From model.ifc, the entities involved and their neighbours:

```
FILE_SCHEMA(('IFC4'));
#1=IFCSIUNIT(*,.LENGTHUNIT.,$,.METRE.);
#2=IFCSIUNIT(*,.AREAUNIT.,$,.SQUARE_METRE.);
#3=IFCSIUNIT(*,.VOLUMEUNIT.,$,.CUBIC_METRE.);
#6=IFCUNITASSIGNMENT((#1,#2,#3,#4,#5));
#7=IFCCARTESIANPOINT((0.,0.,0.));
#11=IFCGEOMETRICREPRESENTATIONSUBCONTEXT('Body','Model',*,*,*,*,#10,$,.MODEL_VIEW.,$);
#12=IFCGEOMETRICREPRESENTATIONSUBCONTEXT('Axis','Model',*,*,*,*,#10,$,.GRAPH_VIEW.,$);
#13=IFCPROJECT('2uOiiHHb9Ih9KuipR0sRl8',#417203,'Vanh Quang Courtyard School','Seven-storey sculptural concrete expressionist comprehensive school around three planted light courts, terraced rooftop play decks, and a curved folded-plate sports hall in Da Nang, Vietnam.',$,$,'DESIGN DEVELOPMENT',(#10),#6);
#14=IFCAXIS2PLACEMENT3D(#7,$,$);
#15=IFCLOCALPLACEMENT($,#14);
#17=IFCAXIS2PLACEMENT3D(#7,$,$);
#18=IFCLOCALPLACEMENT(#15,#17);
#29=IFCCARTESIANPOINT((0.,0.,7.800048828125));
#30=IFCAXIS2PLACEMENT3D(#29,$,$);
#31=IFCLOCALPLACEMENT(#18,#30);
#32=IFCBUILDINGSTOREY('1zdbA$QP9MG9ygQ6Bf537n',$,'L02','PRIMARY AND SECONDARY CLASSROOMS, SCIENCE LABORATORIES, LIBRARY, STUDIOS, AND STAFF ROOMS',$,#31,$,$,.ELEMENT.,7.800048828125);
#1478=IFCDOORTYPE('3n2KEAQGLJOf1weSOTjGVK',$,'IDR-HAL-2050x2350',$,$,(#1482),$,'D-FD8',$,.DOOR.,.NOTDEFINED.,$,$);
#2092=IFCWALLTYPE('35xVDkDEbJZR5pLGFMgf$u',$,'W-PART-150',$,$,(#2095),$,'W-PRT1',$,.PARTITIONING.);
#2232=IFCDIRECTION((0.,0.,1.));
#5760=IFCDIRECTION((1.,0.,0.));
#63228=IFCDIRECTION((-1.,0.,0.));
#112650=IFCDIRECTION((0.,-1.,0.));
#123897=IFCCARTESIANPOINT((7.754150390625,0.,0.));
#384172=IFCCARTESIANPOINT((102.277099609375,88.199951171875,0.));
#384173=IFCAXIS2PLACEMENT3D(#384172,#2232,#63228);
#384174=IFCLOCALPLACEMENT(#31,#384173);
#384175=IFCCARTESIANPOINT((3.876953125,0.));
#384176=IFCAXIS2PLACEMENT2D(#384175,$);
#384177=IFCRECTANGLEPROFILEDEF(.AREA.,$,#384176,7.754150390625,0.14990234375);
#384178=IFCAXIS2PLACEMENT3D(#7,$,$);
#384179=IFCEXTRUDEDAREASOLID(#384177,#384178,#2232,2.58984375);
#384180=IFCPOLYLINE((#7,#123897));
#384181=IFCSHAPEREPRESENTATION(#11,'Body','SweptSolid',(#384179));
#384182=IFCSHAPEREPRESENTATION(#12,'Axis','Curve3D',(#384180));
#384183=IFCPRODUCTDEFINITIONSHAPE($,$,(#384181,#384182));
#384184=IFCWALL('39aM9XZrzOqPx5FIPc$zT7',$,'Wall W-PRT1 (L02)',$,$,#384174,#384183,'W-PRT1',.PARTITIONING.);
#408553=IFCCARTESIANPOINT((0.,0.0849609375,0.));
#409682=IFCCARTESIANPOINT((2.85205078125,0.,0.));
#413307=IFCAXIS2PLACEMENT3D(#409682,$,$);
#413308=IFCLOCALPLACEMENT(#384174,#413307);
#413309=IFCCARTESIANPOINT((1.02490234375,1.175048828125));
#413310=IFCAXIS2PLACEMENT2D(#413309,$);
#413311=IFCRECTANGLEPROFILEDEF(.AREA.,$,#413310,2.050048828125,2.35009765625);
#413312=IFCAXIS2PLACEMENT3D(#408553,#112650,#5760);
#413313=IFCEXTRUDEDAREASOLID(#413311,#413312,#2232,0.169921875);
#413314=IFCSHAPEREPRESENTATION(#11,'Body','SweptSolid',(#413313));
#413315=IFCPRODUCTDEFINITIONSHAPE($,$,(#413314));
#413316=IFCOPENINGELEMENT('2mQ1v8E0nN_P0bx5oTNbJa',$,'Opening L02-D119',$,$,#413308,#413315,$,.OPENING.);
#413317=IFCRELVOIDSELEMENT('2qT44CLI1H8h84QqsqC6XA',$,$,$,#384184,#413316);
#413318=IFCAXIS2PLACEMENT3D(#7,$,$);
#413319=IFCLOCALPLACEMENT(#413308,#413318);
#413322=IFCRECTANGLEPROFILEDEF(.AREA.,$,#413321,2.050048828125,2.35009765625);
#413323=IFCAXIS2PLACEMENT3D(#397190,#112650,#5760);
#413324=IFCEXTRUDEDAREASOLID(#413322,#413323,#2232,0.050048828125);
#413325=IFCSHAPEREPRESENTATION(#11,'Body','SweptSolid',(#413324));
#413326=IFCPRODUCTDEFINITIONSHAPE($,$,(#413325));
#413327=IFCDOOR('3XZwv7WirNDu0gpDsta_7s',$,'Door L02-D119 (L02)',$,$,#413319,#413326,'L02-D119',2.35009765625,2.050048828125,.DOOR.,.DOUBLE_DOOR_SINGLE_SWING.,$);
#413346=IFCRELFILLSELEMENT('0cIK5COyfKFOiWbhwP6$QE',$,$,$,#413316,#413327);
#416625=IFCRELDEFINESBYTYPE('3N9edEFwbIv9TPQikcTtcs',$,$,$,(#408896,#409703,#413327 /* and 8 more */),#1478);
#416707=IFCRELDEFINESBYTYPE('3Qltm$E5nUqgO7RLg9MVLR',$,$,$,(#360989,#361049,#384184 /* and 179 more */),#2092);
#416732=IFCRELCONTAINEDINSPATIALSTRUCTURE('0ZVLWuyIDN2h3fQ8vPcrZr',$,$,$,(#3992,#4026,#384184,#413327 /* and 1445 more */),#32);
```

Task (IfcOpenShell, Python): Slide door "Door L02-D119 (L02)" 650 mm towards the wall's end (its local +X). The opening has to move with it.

```python
import ifcopenshell
import ifcopenshell.api.geometry
import ifcopenshell.util.placement

model = ifcopenshell.open("model.ifc")

door = model.by_guid("3XZwv7WirNDu0gpDsta_7s")
opening = door.FillsVoids[0].RelatingOpeningElement
wall = opening.VoidsElements[0].RelatingBuildingElement

wall_matrix = ifcopenshell.util.placement.get_local_placement(wall.ObjectPlacement)
shift = wall_matrix[:3, 0] * 0.65
before = ifcopenshell.util.placement.get_local_placement(door.ObjectPlacement)[:3, 3].copy()

# The door is placed relative to its opening, so it follows when the opening moves.
matrix = ifcopenshell.util.placement.get_local_placement(opening.ObjectPlacement)
matrix[:3, 3] += shift
ifcopenshell.api.geometry.edit_object_placement(
    model, product=opening, matrix=matrix, is_si=False, should_transform_children=True
)

after = ifcopenshell.util.placement.get_local_placement(door.ObjectPlacement)[:3, 3]
print("door moved by", (after - before).round(3) + 0.0)

model.write("model_edited.ifc")
```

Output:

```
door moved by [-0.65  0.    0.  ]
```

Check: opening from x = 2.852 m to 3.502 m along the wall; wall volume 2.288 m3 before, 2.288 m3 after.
